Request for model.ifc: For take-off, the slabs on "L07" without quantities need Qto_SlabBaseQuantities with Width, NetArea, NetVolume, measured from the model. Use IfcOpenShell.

First a look at what the model holds.

```python
import ifcopenshell
import ifcopenshell.util.element
import ifcopenshell.util.unit

model = ifcopenshell.open("model.ifc")
print(model.schema)
for unit_type in ("LENGTHUNIT", "AREAUNIT", "VOLUMEUNIT"):
    print(unit_type, ifcopenshell.util.unit.calculate_unit_scale(model, unit_type))
storey = next(s for s in model.by_type("IfcBuildingStorey") if s.Name == "L07")
slabs = [e for e in ifcopenshell.util.element.get_decomposition(storey) if e.is_a("IfcSlab")]
for e in sorted(slabs, key=lambda e: e.id()):
    print(e.id(), e.is_a(), e.Name, list(ifcopenshell.util.element.get_psets(e, qtos_only=True)), sep=" | ")
```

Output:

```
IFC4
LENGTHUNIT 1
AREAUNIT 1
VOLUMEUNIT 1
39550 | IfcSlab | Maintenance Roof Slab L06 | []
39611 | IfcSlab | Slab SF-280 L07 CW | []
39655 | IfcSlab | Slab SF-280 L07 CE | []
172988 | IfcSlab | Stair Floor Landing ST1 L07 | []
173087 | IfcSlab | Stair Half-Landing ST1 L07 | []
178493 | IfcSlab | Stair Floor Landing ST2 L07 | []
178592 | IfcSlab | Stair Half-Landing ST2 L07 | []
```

```python
import ifcopenshell
import ifcopenshell.api.pset
import ifcopenshell.geom
import ifcopenshell.util.element
import ifcopenshell.util.shape
import ifcopenshell.util.unit

model = ifcopenshell.open("model.ifc")
unit_scale = ifcopenshell.util.unit.calculate_unit_scale(model)
area_scale = ifcopenshell.util.unit.calculate_unit_scale(model, "AREAUNIT")
volume_scale = ifcopenshell.util.unit.calculate_unit_scale(model, "VOLUMEUNIT")
settings = ifcopenshell.geom.settings()

storey = next(s for s in model.by_type("IfcBuildingStorey") if s.Name == "L07")
slabs = [e for e in ifcopenshell.util.element.get_decomposition(storey) if e.is_a("IfcSlab")]

for e in sorted(slabs, key=lambda e: e.id()):
    if ifcopenshell.util.element.get_psets(e, qtos_only=True, should_inherit=False):
        continue
    # Geometry comes back in metres, in the element's own axes.
    shape = ifcopenshell.geom.create_shape(settings, e)
    values = {
        "Width": ifcopenshell.util.shape.get_z(shape.geometry) / unit_scale,
        "NetArea": ifcopenshell.util.shape.get_footprint_area(shape.geometry) / area_scale,
        "NetVolume": ifcopenshell.util.shape.get_volume(shape.geometry) / volume_scale,
    }
    qto = ifcopenshell.api.pset.add_qto(model, product=e, name="Qto_SlabBaseQuantities")
    ifcopenshell.api.pset.edit_qto(model, qto=qto, properties=values)
    print(e.id(), {k: round(v, 3) for k, v in values.items()})

model.write("model_edited.ifc")
```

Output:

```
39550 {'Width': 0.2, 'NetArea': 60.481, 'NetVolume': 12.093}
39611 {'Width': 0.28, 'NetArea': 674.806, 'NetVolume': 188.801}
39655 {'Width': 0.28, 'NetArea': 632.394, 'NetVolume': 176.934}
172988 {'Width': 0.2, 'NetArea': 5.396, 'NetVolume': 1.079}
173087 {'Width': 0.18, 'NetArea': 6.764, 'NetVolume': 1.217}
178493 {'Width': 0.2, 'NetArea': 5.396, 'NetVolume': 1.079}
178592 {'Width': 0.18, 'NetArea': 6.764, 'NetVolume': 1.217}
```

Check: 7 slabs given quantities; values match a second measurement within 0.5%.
